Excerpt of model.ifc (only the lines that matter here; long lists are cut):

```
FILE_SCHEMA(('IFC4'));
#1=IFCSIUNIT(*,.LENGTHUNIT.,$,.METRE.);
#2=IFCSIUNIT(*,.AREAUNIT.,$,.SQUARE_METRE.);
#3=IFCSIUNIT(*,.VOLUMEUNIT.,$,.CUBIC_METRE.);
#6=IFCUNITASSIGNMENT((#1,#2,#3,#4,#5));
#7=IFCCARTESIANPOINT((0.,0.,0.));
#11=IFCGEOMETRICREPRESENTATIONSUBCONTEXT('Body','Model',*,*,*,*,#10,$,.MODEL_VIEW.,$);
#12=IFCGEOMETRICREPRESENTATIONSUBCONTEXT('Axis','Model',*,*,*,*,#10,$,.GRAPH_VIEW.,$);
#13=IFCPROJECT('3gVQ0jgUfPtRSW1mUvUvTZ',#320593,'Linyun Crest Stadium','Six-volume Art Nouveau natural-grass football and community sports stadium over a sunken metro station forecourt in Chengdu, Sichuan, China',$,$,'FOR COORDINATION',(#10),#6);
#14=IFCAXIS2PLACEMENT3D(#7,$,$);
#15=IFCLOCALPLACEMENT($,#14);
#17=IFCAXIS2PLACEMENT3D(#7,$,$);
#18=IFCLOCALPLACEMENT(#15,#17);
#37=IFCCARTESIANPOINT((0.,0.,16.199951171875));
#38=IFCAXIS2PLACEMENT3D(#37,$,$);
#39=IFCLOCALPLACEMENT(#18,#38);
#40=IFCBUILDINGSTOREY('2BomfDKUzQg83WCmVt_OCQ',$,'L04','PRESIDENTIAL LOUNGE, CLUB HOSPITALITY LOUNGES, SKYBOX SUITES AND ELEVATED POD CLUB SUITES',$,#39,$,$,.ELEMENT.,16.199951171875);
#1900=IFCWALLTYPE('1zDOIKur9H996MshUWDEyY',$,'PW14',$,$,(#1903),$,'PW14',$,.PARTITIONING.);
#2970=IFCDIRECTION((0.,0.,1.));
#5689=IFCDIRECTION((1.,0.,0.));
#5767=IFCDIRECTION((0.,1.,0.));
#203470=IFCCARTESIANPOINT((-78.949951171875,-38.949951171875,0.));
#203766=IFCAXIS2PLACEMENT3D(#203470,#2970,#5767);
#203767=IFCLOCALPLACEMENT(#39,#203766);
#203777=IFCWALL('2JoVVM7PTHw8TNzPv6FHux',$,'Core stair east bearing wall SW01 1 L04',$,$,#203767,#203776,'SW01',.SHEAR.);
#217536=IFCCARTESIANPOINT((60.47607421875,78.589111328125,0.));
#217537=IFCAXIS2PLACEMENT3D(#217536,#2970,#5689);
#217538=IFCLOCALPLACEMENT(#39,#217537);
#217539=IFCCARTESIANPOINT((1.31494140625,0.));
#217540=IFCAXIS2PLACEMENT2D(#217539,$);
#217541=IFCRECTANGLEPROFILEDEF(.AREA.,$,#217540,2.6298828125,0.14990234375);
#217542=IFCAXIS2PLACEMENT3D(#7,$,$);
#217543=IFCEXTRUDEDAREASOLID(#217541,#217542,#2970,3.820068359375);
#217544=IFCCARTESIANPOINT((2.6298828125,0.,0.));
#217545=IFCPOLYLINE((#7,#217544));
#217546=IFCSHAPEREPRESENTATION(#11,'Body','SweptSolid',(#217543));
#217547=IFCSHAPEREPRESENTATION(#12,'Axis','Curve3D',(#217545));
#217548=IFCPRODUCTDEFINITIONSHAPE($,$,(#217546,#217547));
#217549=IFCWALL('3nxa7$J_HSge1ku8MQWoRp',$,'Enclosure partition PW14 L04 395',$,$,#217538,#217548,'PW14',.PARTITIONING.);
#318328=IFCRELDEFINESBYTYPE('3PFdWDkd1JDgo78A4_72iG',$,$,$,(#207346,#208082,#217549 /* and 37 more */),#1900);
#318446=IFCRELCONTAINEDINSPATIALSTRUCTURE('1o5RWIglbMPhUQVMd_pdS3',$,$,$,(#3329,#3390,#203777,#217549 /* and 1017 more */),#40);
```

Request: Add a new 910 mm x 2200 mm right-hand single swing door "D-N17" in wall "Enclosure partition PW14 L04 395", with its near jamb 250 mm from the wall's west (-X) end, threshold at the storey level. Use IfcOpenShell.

```python
import numpy as np
import ifcopenshell
import ifcopenshell.api.feature
import ifcopenshell.api.geometry
import ifcopenshell.api.root
import ifcopenshell.api.spatial
import ifcopenshell.geom
import ifcopenshell.util.element
import ifcopenshell.util.placement
import ifcopenshell.util.representation
import ifcopenshell.util.shape
import ifcopenshell.util.unit

model = ifcopenshell.open("model.ifc")
unit_scale = ifcopenshell.util.unit.calculate_unit_scale(model)
settings = ifcopenshell.geom.settings()


def volume(element):
    """Net volume in cubic metres, openings subtracted."""
    shape = ifcopenshell.geom.create_shape(settings, element)
    return ifcopenshell.util.shape.get_volume(shape.geometry)


wall = model.by_id(217549)
storey = ifcopenshell.util.element.get_container(wall, ifc_class="IfcBuildingStorey")
context = ifcopenshell.util.representation.get_context(model, "Model", "Body", "MODEL_VIEW")
before = volume(wall)

width, height, from_end, sill = 0.91, 2.2, 0.25, 0.0  # metres

# The wall runs along its own X axis, and the end named is its -X end.
wall_shape = ifcopenshell.geom.create_shape(settings, wall)
x, y, z = ifcopenshell.util.shape.get_vertices(wall_shape.geometry).T
start = x.min() + from_end
face, thickness = float(y.min()), float(y.max() - y.min())
wall_matrix = ifcopenshell.util.placement.get_local_placement(wall.ObjectPlacement)
level = ifcopenshell.util.placement.get_local_placement(storey.ObjectPlacement)[2, 3]


def in_wall(x, y):
    """Placement at x, y metres in the wall's axes, at sill height."""
    matrix = wall_matrix.copy()
    matrix[:, 3] = wall_matrix @ np.array([x / unit_scale, y / unit_scale, 0.0, 1.0])
    matrix[2, 3] = level + sill / unit_scale
    return matrix


# Opening: a box that overshoots both wall faces by 50 mm.
opening = ifcopenshell.api.root.create_entity(model, ifc_class="IfcOpeningElement", predefined_type="OPENING")
box = ifcopenshell.api.geometry.add_wall_representation(
    model, context=context, length=width, height=height, thickness=thickness + 0.1
)
ifcopenshell.api.geometry.assign_representation(model, product=opening, representation=box)
ifcopenshell.api.geometry.edit_object_placement(model, product=opening, matrix=in_wall(start, face - 0.05), is_si=False)
ifcopenshell.api.feature.add_feature(model, feature=opening, element=wall)

door = ifcopenshell.api.root.create_entity(model, ifc_class="IfcDoor", name="D-N17", predefined_type="DOOR")
door.OverallWidth, door.OverallHeight = width / unit_scale, height / unit_scale
door.OperationType = "SINGLE_SWING_RIGHT"
body = ifcopenshell.api.geometry.add_door_representation(
    model,
    context=context,
    overall_width=door.OverallWidth,
    overall_height=door.OverallHeight,
    operation_type="SINGLE_SWING_RIGHT",
    lining_properties={"LiningDepth": thickness / unit_scale, "ThresholdDepth": thickness / unit_scale},
)
ifcopenshell.api.geometry.assign_representation(model, product=door, representation=body)
ifcopenshell.api.spatial.assign_container(model, products=[door], relating_structure=storey)
ifcopenshell.api.feature.add_filling(model, opening=opening, element=door)

# The lining spans the wall, so the door starts at the wall face.
ifcopenshell.api.geometry.edit_object_placement(model, product=door, matrix=in_wall(start, face), is_si=False)

after = volume(wall)

print(f"wall volume {before:.3f} -> {after:.3f} m3")

model.write("model_edited.ifc")
```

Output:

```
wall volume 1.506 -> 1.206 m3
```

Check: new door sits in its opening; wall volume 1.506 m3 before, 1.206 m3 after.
